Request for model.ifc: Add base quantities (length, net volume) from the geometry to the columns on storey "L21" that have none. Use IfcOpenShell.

First a look at what the model holds.

```python
import ifcopenshell
import ifcopenshell.util.element
import ifcopenshell.util.unit

model = ifcopenshell.open("model.ifc")
print(model.schema)
for unit_type in ("LENGTHUNIT", "AREAUNIT", "VOLUMEUNIT"):
    print(unit_type, ifcopenshell.util.unit.calculate_unit_scale(model, unit_type))
storey = next(s for s in model.by_type("IfcBuildingStorey") if s.Name == "L21")
columns = [e for e in ifcopenshell.util.element.get_decomposition(storey) if e.is_a("IfcColumn")]
for e in sorted(columns, key=lambda e: e.id()):
    print(e.id(), e.is_a(), e.Name, list(ifcopenshell.util.element.get_psets(e, qtos_only=True)), sep=" | ")
```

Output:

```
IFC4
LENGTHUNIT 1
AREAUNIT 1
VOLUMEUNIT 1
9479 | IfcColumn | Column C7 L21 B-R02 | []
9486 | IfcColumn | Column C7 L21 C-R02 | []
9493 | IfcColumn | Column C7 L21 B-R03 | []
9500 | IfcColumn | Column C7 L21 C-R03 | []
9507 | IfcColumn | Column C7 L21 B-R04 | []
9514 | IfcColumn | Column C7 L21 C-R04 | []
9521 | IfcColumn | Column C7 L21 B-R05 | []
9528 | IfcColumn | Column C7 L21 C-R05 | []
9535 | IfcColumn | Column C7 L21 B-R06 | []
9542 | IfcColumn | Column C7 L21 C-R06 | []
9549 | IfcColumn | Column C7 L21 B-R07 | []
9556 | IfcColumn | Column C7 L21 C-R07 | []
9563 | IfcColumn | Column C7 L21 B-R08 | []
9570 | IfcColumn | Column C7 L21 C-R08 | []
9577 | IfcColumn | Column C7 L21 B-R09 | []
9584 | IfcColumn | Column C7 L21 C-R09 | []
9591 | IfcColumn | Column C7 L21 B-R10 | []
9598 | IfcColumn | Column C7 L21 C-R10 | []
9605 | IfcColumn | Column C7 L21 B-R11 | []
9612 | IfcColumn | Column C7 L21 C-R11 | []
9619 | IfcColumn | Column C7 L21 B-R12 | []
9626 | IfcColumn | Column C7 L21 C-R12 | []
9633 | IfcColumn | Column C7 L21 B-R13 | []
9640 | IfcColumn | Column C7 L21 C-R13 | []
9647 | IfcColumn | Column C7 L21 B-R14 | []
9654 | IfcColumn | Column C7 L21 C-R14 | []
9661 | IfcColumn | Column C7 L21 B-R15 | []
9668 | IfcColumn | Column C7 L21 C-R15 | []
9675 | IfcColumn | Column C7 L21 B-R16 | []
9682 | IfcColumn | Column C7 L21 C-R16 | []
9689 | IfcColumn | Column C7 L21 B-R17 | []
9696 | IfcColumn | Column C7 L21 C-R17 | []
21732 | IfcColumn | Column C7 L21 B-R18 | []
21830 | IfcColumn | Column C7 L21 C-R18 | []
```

```python
import ifcopenshell
import ifcopenshell.api.pset
import ifcopenshell.geom
import ifcopenshell.util.element
import ifcopenshell.util.shape
import ifcopenshell.util.unit

model = ifcopenshell.open("model.ifc")
unit_scale = ifcopenshell.util.unit.calculate_unit_scale(model)
volume_scale = ifcopenshell.util.unit.calculate_unit_scale(model, "VOLUMEUNIT")
settings = ifcopenshell.geom.settings()

storey = next(s for s in model.by_type("IfcBuildingStorey") if s.Name == "L21")
columns = [e for e in ifcopenshell.util.element.get_decomposition(storey) if e.is_a("IfcColumn")]

for e in sorted(columns, key=lambda e: e.id()):
    if ifcopenshell.util.element.get_psets(e, qtos_only=True, should_inherit=False):
        continue
    # Geometry comes back in metres, in the element's own axes.
    shape = ifcopenshell.geom.create_shape(settings, e)
    values = {
        "Length": ifcopenshell.util.shape.get_z(shape.geometry) / unit_scale,
        "NetVolume": ifcopenshell.util.shape.get_volume(shape.geometry) / volume_scale,
    }
    qto = ifcopenshell.api.pset.add_qto(model, product=e, name="Qto_ColumnBaseQuantities")
    ifcopenshell.api.pset.edit_qto(model, qto=qto, properties=values)
    print(e.id(), {k: round(v, 3) for k, v in values.items()})

model.write("model_edited.ifc")
```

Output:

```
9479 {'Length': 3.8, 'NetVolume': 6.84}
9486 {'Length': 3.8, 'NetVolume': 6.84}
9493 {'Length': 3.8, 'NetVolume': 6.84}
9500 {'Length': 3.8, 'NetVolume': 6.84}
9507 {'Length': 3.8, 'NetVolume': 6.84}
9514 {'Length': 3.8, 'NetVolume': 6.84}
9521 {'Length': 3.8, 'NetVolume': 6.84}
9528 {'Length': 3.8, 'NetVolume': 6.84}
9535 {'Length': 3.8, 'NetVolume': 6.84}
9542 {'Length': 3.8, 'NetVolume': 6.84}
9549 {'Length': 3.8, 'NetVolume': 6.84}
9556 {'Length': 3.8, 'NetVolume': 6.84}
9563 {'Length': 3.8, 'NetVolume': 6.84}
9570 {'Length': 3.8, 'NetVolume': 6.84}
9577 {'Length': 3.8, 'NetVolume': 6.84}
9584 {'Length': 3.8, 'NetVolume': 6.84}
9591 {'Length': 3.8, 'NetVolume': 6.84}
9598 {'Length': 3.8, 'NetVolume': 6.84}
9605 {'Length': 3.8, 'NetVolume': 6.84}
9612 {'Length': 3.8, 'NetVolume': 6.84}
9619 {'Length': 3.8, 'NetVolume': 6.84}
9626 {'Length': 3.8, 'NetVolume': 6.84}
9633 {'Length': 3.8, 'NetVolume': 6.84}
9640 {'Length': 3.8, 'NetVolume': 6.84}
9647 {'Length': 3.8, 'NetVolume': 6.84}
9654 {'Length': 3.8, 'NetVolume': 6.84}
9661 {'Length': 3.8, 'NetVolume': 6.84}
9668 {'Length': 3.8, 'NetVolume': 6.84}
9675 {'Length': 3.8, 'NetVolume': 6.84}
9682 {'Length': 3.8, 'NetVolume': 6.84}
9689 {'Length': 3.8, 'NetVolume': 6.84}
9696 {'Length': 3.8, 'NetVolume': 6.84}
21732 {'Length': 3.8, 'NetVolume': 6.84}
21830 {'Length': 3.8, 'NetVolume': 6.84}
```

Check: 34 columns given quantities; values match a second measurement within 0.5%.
